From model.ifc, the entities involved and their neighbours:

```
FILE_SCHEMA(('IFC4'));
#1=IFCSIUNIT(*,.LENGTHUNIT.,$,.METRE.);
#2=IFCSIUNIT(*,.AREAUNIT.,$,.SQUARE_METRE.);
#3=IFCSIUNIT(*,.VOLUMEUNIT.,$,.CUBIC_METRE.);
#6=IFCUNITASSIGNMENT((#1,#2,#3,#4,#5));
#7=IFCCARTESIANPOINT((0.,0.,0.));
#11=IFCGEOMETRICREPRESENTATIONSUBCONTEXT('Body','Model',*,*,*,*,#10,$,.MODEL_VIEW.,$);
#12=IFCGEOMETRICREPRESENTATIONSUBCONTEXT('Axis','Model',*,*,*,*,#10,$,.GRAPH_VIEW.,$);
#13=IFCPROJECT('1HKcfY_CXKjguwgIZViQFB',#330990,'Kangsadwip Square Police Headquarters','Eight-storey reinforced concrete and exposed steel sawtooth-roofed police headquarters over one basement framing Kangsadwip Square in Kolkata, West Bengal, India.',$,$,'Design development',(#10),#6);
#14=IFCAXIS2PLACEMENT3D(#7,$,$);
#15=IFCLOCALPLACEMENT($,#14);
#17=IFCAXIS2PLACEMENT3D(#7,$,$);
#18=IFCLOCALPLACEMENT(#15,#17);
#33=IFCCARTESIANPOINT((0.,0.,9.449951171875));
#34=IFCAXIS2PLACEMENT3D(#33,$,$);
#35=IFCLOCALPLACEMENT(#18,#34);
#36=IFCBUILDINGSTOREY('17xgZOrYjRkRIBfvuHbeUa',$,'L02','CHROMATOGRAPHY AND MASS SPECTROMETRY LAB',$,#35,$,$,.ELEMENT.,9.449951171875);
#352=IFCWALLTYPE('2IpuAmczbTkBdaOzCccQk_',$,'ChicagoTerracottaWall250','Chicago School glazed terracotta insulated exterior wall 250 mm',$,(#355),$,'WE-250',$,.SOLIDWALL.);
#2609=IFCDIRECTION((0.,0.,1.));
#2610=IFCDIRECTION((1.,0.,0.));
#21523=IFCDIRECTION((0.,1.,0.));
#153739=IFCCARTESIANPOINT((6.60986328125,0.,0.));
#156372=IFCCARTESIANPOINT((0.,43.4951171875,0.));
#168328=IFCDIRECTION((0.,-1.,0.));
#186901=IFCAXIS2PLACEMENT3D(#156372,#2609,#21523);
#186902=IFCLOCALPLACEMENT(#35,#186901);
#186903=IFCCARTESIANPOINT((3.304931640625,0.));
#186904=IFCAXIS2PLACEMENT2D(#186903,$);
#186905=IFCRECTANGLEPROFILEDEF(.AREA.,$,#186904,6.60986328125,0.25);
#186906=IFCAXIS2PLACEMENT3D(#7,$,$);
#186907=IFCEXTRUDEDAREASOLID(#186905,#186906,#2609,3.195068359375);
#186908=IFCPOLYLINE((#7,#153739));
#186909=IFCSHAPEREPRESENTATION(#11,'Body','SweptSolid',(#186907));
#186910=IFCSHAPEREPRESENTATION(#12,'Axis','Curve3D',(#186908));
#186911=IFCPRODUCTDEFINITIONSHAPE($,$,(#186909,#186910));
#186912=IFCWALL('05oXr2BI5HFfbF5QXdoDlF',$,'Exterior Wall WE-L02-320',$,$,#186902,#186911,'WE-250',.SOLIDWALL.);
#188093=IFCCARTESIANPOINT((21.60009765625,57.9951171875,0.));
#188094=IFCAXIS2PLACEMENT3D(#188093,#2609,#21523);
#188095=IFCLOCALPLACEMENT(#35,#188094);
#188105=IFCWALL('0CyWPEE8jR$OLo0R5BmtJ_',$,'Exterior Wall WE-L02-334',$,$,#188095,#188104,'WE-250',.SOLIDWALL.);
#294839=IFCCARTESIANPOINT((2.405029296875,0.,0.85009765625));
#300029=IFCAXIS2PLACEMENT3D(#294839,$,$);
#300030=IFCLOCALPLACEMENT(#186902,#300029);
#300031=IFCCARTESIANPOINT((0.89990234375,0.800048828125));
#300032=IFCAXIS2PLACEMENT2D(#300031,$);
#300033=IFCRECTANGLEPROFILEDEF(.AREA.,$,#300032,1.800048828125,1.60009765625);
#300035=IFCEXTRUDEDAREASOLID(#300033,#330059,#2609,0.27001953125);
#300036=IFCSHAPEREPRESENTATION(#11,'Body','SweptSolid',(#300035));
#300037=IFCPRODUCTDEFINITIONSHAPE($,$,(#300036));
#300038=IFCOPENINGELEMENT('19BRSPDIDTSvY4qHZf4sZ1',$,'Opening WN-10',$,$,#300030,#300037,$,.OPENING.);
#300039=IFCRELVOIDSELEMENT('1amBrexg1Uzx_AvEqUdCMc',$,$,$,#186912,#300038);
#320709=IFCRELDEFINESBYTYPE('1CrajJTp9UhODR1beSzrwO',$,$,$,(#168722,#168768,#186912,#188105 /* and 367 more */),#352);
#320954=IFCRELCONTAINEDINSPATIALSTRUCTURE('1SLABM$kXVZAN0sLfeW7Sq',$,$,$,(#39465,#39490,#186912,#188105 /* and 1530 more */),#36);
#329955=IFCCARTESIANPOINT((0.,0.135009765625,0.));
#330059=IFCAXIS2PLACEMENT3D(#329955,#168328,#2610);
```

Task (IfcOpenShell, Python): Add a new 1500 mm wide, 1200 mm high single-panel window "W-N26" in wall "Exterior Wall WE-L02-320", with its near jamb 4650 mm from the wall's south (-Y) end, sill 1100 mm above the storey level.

```python
import numpy as np
import ifcopenshell
import ifcopenshell.api.feature
import ifcopenshell.api.geometry
import ifcopenshell.api.root
import ifcopenshell.api.spatial
import ifcopenshell.geom
import ifcopenshell.util.element
import ifcopenshell.util.placement
import ifcopenshell.util.representation
import ifcopenshell.util.shape
import ifcopenshell.util.unit

model = ifcopenshell.open("model.ifc")
unit_scale = ifcopenshell.util.unit.calculate_unit_scale(model)
settings = ifcopenshell.geom.settings()


def volume(element):
    """Net volume in cubic metres, openings subtracted."""
    shape = ifcopenshell.geom.create_shape(settings, element)
    return ifcopenshell.util.shape.get_volume(shape.geometry)


wall = model.by_guid("05oXr2BI5HFfbF5QXdoDlF")
storey = ifcopenshell.util.element.get_container(wall, ifc_class="IfcBuildingStorey")
context = ifcopenshell.util.representation.get_context(model, "Model", "Body", "MODEL_VIEW")
before = volume(wall)

width, height, from_end, sill = 1.5, 1.2, 4.65, 1.1  # metres

# The wall runs along its own X axis, and the end named is its -X end.
wall_shape = ifcopenshell.geom.create_shape(settings, wall)
x, y, z = ifcopenshell.util.shape.get_vertices(wall_shape.geometry).T
start = x.min() + from_end
face, thickness = float(y.min()), float(y.max() - y.min())
wall_matrix = ifcopenshell.util.placement.get_local_placement(wall.ObjectPlacement)
level = ifcopenshell.util.placement.get_local_placement(storey.ObjectPlacement)[2, 3]


def in_wall(x, y):
    """Placement at x, y metres in the wall's axes, at sill height."""
    matrix = wall_matrix.copy()
    matrix[:, 3] = wall_matrix @ np.array([x / unit_scale, y / unit_scale, 0.0, 1.0])
    matrix[2, 3] = level + sill / unit_scale
    return matrix


# Opening: a box that overshoots both wall faces by 50 mm.
opening = ifcopenshell.api.root.create_entity(model, ifc_class="IfcOpeningElement", predefined_type="OPENING")
box = ifcopenshell.api.geometry.add_wall_representation(
    model, context=context, length=width, height=height, thickness=thickness + 0.1
)
ifcopenshell.api.geometry.assign_representation(model, product=opening, representation=box)
ifcopenshell.api.geometry.edit_object_placement(model, product=opening, matrix=in_wall(start, face - 0.05), is_si=False)
ifcopenshell.api.feature.add_feature(model, feature=opening, element=wall)

window = ifcopenshell.api.root.create_entity(model, ifc_class="IfcWindow", name="W-N26", predefined_type="WINDOW")
window.OverallWidth, window.OverallHeight = width / unit_scale, height / unit_scale
window.PartitioningType = "SINGLE_PANEL"
body = ifcopenshell.api.geometry.add_window_representation(
    model,
    context=context,
    overall_width=window.OverallWidth,
    overall_height=window.OverallHeight,
    partition_type="SINGLE_PANEL",
)
ifcopenshell.api.geometry.assign_representation(model, product=window, representation=body)
ifcopenshell.api.spatial.assign_container(model, products=[window], relating_structure=storey)
ifcopenshell.api.feature.add_filling(model, opening=opening, element=window)

# Centre the window in the wall's thickness.
ifcopenshell.api.geometry.edit_object_placement(model, product=window, matrix=in_wall(start, face), is_si=False)
window_shape = ifcopenshell.geom.create_shape(settings, window)
depth = ifcopenshell.util.shape.get_vertices(window_shape.geometry)[:, 1]
offset = face + thickness / 2 - (depth.min() + depth.max()) / 2
ifcopenshell.api.geometry.edit_object_placement(model, product=window, matrix=in_wall(start, offset), is_si=False)

after = volume(wall)

print(f"wall volume {before:.3f} -> {after:.3f} m3")

model.write("model_v2.ifc")
```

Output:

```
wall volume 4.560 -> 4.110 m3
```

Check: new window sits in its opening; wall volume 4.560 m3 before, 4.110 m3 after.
